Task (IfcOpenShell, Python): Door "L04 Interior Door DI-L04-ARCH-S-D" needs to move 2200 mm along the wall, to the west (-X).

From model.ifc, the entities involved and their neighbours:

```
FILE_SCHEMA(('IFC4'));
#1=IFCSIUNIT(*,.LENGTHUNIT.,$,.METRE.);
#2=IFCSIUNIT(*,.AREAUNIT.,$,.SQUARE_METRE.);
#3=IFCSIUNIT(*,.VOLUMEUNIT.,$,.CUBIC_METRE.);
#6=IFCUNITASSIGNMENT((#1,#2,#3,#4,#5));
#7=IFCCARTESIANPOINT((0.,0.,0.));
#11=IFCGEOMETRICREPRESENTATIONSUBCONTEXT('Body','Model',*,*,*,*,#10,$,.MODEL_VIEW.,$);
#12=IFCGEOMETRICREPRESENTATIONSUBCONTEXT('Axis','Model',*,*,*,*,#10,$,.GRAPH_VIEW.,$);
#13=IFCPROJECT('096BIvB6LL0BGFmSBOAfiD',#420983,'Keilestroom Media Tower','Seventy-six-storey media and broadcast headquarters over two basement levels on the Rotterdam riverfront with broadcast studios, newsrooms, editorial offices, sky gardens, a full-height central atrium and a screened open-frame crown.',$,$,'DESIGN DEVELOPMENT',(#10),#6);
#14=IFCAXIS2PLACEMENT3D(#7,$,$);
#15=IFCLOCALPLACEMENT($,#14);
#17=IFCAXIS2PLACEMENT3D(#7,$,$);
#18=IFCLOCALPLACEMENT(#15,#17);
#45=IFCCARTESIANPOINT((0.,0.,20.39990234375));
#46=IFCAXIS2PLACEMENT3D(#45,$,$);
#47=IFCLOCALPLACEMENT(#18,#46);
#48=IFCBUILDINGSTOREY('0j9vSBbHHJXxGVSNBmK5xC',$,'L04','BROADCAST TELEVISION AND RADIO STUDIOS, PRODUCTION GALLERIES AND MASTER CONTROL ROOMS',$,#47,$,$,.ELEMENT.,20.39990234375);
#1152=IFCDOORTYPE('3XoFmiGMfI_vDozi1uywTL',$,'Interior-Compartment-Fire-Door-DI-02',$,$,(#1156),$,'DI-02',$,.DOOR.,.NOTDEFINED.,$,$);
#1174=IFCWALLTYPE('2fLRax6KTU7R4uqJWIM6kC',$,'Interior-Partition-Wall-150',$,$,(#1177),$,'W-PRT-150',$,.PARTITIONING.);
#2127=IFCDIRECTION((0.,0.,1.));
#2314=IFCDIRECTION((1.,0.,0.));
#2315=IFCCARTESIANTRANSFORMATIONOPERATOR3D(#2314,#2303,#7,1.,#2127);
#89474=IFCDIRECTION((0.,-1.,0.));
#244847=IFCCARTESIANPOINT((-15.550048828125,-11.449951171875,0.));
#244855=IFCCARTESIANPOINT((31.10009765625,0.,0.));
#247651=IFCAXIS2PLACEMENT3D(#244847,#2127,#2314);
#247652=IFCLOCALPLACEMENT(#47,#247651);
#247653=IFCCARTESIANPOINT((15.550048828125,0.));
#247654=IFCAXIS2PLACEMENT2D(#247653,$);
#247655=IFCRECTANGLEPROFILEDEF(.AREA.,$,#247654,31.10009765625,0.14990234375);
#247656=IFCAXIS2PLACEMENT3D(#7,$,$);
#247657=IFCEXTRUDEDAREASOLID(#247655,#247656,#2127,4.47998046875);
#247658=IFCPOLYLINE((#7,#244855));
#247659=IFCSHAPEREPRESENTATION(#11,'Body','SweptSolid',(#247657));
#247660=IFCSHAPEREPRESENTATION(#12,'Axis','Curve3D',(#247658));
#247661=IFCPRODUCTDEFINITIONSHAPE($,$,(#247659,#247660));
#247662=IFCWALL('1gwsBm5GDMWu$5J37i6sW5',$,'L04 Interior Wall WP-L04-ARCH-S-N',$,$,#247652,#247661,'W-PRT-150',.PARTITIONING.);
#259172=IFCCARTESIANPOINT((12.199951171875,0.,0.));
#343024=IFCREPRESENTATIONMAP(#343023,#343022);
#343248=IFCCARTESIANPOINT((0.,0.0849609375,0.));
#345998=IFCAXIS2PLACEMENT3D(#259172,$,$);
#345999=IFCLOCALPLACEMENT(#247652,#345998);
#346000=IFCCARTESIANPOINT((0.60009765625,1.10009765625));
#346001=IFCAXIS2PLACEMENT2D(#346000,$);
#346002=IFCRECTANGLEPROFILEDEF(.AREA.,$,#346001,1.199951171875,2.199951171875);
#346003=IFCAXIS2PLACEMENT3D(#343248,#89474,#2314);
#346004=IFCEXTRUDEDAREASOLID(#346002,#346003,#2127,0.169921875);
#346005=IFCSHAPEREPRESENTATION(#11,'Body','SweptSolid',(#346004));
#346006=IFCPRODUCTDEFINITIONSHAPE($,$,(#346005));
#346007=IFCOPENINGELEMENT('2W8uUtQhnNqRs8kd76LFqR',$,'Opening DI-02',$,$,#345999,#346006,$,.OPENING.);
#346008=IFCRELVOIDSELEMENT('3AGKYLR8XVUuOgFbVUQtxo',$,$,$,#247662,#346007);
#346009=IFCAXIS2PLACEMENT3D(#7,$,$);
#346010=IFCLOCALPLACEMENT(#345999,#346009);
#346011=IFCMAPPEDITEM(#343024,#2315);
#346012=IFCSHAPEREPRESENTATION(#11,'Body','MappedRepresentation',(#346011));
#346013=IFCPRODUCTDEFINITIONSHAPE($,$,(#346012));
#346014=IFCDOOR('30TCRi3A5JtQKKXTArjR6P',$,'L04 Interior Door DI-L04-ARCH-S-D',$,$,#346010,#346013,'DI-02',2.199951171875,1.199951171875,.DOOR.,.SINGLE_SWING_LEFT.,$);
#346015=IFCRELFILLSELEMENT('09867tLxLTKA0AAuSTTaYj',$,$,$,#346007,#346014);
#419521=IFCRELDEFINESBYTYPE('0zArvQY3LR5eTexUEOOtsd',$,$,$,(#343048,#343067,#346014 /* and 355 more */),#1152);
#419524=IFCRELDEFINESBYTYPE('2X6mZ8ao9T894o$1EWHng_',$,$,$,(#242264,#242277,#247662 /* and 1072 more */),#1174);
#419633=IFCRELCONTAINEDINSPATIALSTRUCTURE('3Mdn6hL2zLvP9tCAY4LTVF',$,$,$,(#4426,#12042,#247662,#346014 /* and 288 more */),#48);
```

```python
import ifcopenshell
import ifcopenshell.api.geometry
import ifcopenshell.util.placement
import ifcopenshell.util.unit

model = ifcopenshell.open("model.ifc")
unit_scale = ifcopenshell.util.unit.calculate_unit_scale(model)

door = model.by_guid("30TCRi3A5JtQKKXTArjR6P")
opening = door.FillsVoids[0].RelatingOpeningElement
wall = opening.VoidsElements[0].RelatingBuildingElement

wall_matrix = ifcopenshell.util.placement.get_local_placement(wall.ObjectPlacement)
shift = wall_matrix[:3, 0] * -2.2 / unit_scale
before = ifcopenshell.util.placement.get_local_placement(door.ObjectPlacement)[:3, 3].copy()

# The door is placed relative to its opening, so it follows when the opening moves.
matrix = ifcopenshell.util.placement.get_local_placement(opening.ObjectPlacement)
matrix[:3, 3] += shift
ifcopenshell.api.geometry.edit_object_placement(
    model, product=opening, matrix=matrix, is_si=False, should_transform_children=True
)

after = ifcopenshell.util.placement.get_local_placement(door.ObjectPlacement)[:3, 3]
print("door moved by", (after - before).round(3) + 0.0)

model.write("model_v2.ifc")
```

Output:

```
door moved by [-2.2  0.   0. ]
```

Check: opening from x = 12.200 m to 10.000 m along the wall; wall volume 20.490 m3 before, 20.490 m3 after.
